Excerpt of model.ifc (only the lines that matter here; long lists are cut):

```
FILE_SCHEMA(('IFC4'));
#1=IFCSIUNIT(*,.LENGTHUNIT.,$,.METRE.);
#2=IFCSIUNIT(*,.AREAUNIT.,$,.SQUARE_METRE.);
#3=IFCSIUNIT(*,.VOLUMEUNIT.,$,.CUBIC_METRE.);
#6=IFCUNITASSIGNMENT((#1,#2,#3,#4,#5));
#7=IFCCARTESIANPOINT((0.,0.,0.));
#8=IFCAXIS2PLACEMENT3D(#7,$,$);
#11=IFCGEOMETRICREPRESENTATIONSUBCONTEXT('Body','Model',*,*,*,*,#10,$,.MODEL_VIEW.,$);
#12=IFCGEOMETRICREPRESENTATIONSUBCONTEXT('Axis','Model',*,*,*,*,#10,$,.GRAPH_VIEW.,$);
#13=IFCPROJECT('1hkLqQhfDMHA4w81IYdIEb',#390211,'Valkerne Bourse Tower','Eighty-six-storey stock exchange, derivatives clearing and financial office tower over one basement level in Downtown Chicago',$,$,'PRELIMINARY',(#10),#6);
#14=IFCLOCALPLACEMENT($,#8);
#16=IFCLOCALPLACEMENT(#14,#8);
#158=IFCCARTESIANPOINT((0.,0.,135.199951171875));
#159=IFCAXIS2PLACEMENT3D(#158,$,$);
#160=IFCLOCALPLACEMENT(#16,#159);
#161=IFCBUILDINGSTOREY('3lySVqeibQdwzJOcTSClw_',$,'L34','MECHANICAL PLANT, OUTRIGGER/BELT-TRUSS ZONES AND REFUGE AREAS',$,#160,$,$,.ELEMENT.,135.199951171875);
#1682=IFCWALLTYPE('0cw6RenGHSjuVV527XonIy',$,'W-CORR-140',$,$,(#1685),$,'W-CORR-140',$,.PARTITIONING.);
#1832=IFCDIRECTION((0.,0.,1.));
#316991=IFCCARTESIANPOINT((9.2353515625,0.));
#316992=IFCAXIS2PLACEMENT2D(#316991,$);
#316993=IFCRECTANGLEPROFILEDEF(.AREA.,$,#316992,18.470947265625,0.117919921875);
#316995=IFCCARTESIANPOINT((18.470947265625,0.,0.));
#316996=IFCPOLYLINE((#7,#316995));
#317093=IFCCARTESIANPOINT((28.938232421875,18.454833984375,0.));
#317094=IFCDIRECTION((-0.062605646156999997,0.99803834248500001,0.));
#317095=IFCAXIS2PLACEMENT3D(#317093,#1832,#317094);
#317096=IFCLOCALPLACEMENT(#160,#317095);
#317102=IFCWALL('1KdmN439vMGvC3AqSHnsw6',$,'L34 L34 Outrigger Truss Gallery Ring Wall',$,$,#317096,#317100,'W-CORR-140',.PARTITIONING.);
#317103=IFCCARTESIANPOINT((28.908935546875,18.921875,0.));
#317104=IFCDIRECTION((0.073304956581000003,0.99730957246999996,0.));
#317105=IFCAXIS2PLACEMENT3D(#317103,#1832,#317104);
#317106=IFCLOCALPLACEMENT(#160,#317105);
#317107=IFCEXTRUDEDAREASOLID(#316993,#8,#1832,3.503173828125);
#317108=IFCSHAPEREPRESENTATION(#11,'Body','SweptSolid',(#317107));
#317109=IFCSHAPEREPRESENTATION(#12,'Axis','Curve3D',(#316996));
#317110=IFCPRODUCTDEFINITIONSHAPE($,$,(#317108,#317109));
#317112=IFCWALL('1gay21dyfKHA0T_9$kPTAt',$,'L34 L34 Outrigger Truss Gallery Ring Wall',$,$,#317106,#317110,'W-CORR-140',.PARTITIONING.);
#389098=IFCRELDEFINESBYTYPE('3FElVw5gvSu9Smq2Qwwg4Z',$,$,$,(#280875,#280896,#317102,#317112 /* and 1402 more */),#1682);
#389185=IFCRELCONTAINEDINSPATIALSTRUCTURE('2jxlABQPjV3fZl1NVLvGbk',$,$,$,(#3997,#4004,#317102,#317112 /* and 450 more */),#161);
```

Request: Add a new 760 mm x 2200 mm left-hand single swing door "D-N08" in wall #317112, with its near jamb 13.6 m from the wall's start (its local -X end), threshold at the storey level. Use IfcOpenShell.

```python
import numpy as np
import ifcopenshell
import ifcopenshell.api.feature
import ifcopenshell.api.geometry
import ifcopenshell.api.root
import ifcopenshell.api.spatial
import ifcopenshell.geom
import ifcopenshell.util.element
import ifcopenshell.util.placement
import ifcopenshell.util.representation
import ifcopenshell.util.shape
import ifcopenshell.util.unit

model = ifcopenshell.open("model.ifc")
unit_scale = ifcopenshell.util.unit.calculate_unit_scale(model)
settings = ifcopenshell.geom.settings()


def volume(element):
    """Net volume in cubic metres, openings subtracted."""
    shape = ifcopenshell.geom.create_shape(settings, element)
    return ifcopenshell.util.shape.get_volume(shape.geometry)


wall = model.by_guid("1gay21dyfKHA0T_9$kPTAt")
storey = ifcopenshell.util.element.get_container(wall, ifc_class="IfcBuildingStorey")
context = ifcopenshell.util.representation.get_context(model, "Model", "Body", "MODEL_VIEW")
before = volume(wall)

width, height, from_end, sill = 0.76, 2.2, 13.6, 0.0  # metres

# The wall runs along its own X axis, and the end named is its -X end.
wall_shape = ifcopenshell.geom.create_shape(settings, wall)
x, y, z = ifcopenshell.util.shape.get_vertices(wall_shape.geometry).T
start = x.min() + from_end
face, thickness = float(y.min()), float(y.max() - y.min())
wall_matrix = ifcopenshell.util.placement.get_local_placement(wall.ObjectPlacement)
level = ifcopenshell.util.placement.get_local_placement(storey.ObjectPlacement)[2, 3]


def in_wall(x, y):
    """Placement at x, y metres in the wall's axes, at sill height."""
    matrix = wall_matrix.copy()
    matrix[:, 3] = wall_matrix @ np.array([x / unit_scale, y / unit_scale, 0.0, 1.0])
    matrix[2, 3] = level + sill / unit_scale
    return matrix


# Opening: a box that overshoots both wall faces by 50 mm.
opening = ifcopenshell.api.root.create_entity(model, ifc_class="IfcOpeningElement", predefined_type="OPENING")
box = ifcopenshell.api.geometry.add_wall_representation(
    model, context=context, length=width, height=height, thickness=thickness + 0.1
)
ifcopenshell.api.geometry.assign_representation(model, product=opening, representation=box)
ifcopenshell.api.geometry.edit_object_placement(model, product=opening, matrix=in_wall(start, face - 0.05), is_si=False)
ifcopenshell.api.feature.add_feature(model, feature=opening, element=wall)

door = ifcopenshell.api.root.create_entity(model, ifc_class="IfcDoor", name="D-N08", predefined_type="DOOR")
door.OverallWidth, door.OverallHeight = width / unit_scale, height / unit_scale
door.OperationType = "SINGLE_SWING_LEFT"
body = ifcopenshell.api.geometry.add_door_representation(
    model,
    context=context,
    overall_width=door.OverallWidth,
    overall_height=door.OverallHeight,
    operation_type="SINGLE_SWING_LEFT",
    lining_properties={"LiningDepth": thickness / unit_scale, "ThresholdDepth": thickness / unit_scale},
)
ifcopenshell.api.geometry.assign_representation(model, product=door, representation=body)
ifcopenshell.api.spatial.assign_container(model, products=[door], relating_structure=storey)
ifcopenshell.api.feature.add_filling(model, opening=opening, element=door)

# The lining spans the wall, so the door starts at the wall face.
ifcopenshell.api.geometry.edit_object_placement(model, product=door, matrix=in_wall(start, face), is_si=False)

after = volume(wall)

print(f"wall volume {before:.3f} -> {after:.3f} m3")

model.write("model_updated.ifc")
```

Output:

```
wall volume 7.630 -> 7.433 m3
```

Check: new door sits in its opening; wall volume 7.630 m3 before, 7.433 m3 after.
